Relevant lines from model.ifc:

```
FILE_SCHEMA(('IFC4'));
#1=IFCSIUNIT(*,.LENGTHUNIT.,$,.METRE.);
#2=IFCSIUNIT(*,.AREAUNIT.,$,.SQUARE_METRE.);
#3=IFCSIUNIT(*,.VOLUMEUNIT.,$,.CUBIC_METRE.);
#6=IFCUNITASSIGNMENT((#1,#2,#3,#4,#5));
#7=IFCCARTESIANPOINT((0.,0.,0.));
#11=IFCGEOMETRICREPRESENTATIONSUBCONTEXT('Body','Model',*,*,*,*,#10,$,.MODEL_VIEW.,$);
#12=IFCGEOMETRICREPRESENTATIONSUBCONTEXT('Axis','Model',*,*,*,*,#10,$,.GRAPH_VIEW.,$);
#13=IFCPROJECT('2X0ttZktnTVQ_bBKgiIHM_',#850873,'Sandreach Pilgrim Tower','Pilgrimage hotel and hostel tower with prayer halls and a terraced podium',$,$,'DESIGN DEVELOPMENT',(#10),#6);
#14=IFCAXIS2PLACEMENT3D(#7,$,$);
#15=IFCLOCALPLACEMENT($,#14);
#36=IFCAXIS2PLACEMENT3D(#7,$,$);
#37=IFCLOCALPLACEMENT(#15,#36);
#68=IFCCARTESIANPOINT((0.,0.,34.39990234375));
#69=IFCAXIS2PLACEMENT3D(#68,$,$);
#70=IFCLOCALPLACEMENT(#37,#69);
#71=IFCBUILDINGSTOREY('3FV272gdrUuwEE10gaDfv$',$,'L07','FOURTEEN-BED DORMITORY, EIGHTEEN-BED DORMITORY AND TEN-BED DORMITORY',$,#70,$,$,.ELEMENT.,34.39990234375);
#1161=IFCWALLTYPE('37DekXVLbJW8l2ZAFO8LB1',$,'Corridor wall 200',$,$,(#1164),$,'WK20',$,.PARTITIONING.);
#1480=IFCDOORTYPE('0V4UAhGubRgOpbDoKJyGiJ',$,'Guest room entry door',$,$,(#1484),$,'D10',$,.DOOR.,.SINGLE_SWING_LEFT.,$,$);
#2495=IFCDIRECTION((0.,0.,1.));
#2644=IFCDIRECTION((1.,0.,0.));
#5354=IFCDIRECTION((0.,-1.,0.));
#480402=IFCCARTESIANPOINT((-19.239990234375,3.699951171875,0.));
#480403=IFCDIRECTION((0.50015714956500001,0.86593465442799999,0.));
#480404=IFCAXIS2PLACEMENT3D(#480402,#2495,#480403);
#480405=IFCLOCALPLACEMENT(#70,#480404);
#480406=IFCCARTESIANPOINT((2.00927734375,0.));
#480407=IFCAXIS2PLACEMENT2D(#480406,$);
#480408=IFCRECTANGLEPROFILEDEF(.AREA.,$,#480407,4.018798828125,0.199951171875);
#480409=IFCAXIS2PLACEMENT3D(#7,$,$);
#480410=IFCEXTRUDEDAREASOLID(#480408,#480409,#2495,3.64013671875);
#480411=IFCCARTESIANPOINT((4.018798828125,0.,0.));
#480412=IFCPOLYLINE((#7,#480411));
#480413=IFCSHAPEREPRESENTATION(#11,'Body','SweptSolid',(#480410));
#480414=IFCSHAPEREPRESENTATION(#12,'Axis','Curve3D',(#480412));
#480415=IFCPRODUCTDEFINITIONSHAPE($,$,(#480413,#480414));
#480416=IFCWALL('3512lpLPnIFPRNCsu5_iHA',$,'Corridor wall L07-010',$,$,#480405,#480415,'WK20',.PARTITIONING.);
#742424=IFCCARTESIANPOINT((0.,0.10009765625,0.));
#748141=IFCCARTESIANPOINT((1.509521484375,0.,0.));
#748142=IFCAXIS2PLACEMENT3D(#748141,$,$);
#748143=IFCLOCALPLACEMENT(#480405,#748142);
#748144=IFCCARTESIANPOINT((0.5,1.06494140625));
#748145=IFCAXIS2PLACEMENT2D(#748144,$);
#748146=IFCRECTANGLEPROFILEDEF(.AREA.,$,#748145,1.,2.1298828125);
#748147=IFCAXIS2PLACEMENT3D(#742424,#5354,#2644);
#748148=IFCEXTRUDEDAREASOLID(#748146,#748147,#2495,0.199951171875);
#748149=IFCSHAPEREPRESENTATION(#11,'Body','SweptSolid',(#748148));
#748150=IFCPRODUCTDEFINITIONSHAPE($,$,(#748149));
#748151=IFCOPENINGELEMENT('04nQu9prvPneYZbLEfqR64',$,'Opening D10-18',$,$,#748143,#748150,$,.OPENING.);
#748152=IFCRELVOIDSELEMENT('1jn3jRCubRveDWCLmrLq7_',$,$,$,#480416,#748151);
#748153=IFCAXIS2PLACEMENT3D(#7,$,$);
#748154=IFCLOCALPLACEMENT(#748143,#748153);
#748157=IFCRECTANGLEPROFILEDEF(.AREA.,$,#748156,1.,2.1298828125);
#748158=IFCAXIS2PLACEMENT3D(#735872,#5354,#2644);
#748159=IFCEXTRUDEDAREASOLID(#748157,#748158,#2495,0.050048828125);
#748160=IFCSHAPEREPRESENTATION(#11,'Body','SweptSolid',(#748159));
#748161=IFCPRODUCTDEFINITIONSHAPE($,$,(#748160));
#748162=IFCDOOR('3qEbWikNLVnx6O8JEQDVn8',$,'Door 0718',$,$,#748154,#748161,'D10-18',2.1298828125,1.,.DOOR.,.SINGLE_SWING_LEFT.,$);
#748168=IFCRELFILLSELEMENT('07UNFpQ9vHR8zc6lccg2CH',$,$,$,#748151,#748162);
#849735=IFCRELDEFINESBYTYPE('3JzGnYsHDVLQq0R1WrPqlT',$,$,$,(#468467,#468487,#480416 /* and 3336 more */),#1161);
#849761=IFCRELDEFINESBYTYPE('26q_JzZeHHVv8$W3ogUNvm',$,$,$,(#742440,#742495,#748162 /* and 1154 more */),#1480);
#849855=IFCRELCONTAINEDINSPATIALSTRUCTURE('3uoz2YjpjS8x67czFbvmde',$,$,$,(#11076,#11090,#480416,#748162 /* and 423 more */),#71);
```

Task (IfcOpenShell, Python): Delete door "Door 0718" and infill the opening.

```python
import ifcopenshell
import ifcopenshell.api.feature
import ifcopenshell.api.root
import ifcopenshell.geom
import ifcopenshell.util.shape

model = ifcopenshell.open("model.ifc")
settings = ifcopenshell.geom.settings()


def volume(element):
    """Net volume in cubic metres, openings subtracted."""
    shape = ifcopenshell.geom.create_shape(settings, element)
    return ifcopenshell.util.shape.get_volume(shape.geometry)


door = model.by_guid("3qEbWikNLVnx6O8JEQDVn8")
opening = door.FillsVoids[0].RelatingOpeningElement
wall = opening.VoidsElements[0].RelatingBuildingElement
before = volume(wall)

ifcopenshell.api.root.remove_product(model, product=door)
ifcopenshell.api.feature.remove_feature(model, feature=opening)

after = volume(wall)

print(f"wall volume {before:.3f} -> {after:.3f} m3")

model.write("model_edited.ifc")
```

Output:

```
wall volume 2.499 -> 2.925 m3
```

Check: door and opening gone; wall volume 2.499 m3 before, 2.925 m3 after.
